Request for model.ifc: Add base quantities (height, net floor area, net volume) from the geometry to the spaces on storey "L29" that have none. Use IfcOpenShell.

First a look at what the model holds.

```python
import ifcopenshell
import ifcopenshell.util.element
import ifcopenshell.util.unit

model = ifcopenshell.open("model.ifc")
print(model.schema)
for unit_type in ("LENGTHUNIT", "AREAUNIT", "VOLUMEUNIT"):
    print(unit_type, ifcopenshell.util.unit.calculate_unit_scale(model, unit_type))
storey = next(s for s in model.by_type("IfcBuildingStorey") if s.Name == "L29")
spaces = [e for e in ifcopenshell.util.element.get_decomposition(storey) if e.is_a("IfcSpace")]
for e in sorted(spaces, key=lambda e: e.id()):
    print(e.id(), e.is_a(), e.Name, list(ifcopenshell.util.element.get_psets(e, qtos_only=True)), sep=" | ")
```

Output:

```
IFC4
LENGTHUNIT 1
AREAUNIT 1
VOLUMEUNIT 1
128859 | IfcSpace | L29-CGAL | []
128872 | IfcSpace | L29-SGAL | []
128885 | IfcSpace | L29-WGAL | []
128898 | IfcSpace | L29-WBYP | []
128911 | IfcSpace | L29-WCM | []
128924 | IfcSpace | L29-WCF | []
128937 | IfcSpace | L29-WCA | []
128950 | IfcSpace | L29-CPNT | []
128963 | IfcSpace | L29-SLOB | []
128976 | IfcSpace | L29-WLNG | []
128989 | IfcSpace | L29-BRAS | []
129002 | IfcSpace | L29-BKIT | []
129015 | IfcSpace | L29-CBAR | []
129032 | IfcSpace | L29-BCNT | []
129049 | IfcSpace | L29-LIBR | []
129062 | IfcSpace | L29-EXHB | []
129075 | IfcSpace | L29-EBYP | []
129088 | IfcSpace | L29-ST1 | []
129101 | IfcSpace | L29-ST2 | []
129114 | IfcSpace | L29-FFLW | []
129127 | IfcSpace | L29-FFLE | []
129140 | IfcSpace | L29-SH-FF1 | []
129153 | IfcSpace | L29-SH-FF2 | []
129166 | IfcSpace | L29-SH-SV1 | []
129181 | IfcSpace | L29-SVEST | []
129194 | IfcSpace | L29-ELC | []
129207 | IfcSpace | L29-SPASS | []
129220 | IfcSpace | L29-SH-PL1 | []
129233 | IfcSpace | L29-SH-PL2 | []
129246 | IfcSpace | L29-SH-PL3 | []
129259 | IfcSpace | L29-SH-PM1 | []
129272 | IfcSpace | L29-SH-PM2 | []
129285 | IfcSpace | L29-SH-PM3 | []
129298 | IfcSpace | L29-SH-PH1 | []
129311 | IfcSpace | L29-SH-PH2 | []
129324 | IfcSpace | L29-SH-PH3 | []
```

```python
import ifcopenshell
import ifcopenshell.api.pset
import ifcopenshell.geom
import ifcopenshell.util.element
import ifcopenshell.util.shape
import ifcopenshell.util.unit

model = ifcopenshell.open("model.ifc")
unit_scale = ifcopenshell.util.unit.calculate_unit_scale(model)
area_scale = ifcopenshell.util.unit.calculate_unit_scale(model, "AREAUNIT")
volume_scale = ifcopenshell.util.unit.calculate_unit_scale(model, "VOLUMEUNIT")
settings = ifcopenshell.geom.settings()

storey = next(s for s in model.by_type("IfcBuildingStorey") if s.Name == "L29")
spaces = [e for e in ifcopenshell.util.element.get_decomposition(storey) if e.is_a("IfcSpace")]

for e in sorted(spaces, key=lambda e: e.id()):
    if ifcopenshell.util.element.get_psets(e, qtos_only=True, should_inherit=False):
        continue
    # Geometry comes back in metres, in the element's own axes.
    shape = ifcopenshell.geom.create_shape(settings, e)
    values = {
        "Height": ifcopenshell.util.shape.get_z(shape.geometry) / unit_scale,
        "NetFloorArea": ifcopenshell.util.shape.get_footprint_area(shape.geometry) / area_scale,
        "NetVolume": ifcopenshell.util.shape.get_volume(shape.geometry) / volume_scale,
    }
    qto = ifcopenshell.api.pset.add_qto(model, product=e, name="Qto_SpaceBaseQuantities")
    ifcopenshell.api.pset.edit_qto(model, qto=qto, properties=values)
    print(e.id(), {k: round(v, 3) for k, v in values.items()})

model.write("model_rev.ifc")
```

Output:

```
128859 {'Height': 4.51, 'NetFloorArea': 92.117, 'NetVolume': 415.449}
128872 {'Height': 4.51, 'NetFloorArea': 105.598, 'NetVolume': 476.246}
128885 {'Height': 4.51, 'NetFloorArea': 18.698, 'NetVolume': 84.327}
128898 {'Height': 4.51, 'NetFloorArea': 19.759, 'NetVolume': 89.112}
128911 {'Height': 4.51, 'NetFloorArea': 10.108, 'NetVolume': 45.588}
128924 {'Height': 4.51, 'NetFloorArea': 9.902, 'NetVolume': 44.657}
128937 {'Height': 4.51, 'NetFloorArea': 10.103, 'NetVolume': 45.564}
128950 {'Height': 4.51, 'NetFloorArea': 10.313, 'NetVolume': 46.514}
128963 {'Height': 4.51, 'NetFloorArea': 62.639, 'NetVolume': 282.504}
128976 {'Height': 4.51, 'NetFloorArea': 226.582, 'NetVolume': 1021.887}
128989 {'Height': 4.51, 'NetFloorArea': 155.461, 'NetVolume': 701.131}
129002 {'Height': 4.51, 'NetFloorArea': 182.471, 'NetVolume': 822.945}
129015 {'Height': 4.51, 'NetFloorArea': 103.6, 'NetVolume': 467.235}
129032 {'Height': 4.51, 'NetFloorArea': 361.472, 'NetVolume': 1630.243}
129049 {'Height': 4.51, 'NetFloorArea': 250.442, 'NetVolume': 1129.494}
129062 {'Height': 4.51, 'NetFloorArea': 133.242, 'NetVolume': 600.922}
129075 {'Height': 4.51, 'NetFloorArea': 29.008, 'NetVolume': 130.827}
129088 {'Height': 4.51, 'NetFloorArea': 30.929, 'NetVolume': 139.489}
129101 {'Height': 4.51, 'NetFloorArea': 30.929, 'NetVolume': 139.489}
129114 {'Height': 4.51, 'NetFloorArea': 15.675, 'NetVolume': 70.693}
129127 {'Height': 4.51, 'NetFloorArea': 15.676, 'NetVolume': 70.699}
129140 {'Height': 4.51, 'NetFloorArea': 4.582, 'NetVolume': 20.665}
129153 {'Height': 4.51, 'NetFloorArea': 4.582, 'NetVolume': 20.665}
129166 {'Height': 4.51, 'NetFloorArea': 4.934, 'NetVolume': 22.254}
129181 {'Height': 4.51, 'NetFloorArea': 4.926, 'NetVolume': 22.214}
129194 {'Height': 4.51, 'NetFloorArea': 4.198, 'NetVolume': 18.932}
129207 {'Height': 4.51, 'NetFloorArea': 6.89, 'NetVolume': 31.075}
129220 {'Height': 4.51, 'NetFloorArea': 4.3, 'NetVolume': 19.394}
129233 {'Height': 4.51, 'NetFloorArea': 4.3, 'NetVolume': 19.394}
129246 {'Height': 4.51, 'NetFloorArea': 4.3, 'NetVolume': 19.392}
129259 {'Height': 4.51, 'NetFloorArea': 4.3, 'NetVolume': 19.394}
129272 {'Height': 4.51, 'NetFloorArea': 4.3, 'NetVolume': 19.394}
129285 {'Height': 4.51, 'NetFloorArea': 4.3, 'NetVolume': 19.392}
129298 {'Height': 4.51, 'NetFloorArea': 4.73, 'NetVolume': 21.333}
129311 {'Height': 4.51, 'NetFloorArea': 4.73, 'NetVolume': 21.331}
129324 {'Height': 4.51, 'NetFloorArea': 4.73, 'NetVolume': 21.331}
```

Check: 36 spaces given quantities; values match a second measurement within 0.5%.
